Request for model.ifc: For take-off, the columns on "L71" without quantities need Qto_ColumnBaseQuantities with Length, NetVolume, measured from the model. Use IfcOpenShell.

First a look at what the model holds.

```python
import ifcopenshell
import ifcopenshell.util.element
import ifcopenshell.util.unit

model = ifcopenshell.open("model.ifc")
print(model.schema)
for unit_type in ("LENGTHUNIT", "AREAUNIT", "VOLUMEUNIT"):
    print(unit_type, ifcopenshell.util.unit.calculate_unit_scale(model, unit_type))
storey = next(s for s in model.by_type("IfcBuildingStorey") if s.Name == "L71")
columns = [e for e in ifcopenshell.util.element.get_decomposition(storey) if e.is_a("IfcColumn")]
for e in sorted(columns, key=lambda e: e.id()):
    print(e.id(), e.is_a(), e.Name, list(ifcopenshell.util.element.get_psets(e, qtos_only=True)), sep=" | ")
```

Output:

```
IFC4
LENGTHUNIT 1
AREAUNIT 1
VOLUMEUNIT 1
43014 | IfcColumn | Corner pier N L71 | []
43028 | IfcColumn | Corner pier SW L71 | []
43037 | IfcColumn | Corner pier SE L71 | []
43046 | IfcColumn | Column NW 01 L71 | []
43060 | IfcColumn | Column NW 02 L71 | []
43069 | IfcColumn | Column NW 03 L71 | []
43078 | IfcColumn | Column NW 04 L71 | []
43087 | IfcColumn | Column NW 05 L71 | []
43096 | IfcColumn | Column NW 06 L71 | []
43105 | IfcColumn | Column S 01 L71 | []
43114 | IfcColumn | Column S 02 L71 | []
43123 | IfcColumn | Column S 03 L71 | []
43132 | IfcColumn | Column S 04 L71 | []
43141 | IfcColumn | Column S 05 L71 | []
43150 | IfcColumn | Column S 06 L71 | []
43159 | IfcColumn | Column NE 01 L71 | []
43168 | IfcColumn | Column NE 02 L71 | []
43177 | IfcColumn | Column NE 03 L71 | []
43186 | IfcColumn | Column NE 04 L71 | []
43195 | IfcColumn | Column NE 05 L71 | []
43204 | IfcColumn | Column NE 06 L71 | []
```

```python
import ifcopenshell
import ifcopenshell.api.pset
import ifcopenshell.geom
import ifcopenshell.util.element
import ifcopenshell.util.shape
import ifcopenshell.util.unit

model = ifcopenshell.open("model.ifc")
unit_scale = ifcopenshell.util.unit.calculate_unit_scale(model)
volume_scale = ifcopenshell.util.unit.calculate_unit_scale(model, "VOLUMEUNIT")
settings = ifcopenshell.geom.settings()

storey = next(s for s in model.by_type("IfcBuildingStorey") if s.Name == "L71")
columns = [e for e in ifcopenshell.util.element.get_decomposition(storey) if e.is_a("IfcColumn")]

for e in sorted(columns, key=lambda e: e.id()):
    if ifcopenshell.util.element.get_psets(e, qtos_only=True, should_inherit=False):
        continue
    # Geometry comes back in metres, in the element's own axes.
    shape = ifcopenshell.geom.create_shape(settings, e)
    values = {
        "Length": ifcopenshell.util.shape.get_z(shape.geometry) / unit_scale,
        "NetVolume": ifcopenshell.util.shape.get_volume(shape.geometry) / volume_scale,
    }
    qto = ifcopenshell.api.pset.add_qto(model, product=e, name="Qto_ColumnBaseQuantities")
    ifcopenshell.api.pset.edit_qto(model, qto=qto, properties=values)
    print(e.id(), {k: round(v, 3) for k, v in values.items()})

model.write("model_v2.ifc")
```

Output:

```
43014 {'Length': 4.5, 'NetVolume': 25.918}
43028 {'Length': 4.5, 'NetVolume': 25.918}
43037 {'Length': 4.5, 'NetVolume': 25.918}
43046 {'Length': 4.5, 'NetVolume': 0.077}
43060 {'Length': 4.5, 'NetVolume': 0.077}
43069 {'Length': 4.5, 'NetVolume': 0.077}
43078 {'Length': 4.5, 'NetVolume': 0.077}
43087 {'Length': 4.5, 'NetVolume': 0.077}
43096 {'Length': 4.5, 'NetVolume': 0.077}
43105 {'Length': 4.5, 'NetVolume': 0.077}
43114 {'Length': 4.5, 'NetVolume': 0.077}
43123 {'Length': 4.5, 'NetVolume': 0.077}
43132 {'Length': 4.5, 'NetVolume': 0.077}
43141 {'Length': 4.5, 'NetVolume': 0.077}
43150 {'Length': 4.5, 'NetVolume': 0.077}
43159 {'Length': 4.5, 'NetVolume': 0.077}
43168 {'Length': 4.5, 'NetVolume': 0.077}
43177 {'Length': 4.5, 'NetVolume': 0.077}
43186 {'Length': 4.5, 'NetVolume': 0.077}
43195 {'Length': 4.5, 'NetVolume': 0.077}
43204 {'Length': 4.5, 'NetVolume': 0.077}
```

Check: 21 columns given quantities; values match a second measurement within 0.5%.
